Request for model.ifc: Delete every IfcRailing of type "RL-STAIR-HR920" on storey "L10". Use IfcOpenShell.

First a look at what the model holds.

```python
import ifcopenshell
import ifcopenshell.util.element

model = ifcopenshell.open("model.ifc")
print(model.schema)
storey = next(s for s in model.by_type("IfcBuildingStorey") if s.Name == "L10")
railings = [e for e in ifcopenshell.util.element.get_decomposition(storey) if e.is_a("IfcRailing")]
seen = {}
for e in railings:
    element_type = ifcopenshell.util.element.get_type(e)
    name = element_type.Name if element_type not in (None, e) else None
    seen[name] = seen.get(name, 0) + 1
for name, count in sorted(seen.items(), key=str):
    print(count, "x", name)
```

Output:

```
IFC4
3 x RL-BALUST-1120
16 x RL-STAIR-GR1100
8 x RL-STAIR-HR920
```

```python
import ifcopenshell
import ifcopenshell.api.root
import ifcopenshell.util.element

model = ifcopenshell.open("model.ifc")

storey = next(s for s in model.by_type("IfcBuildingStorey") if s.Name == "L10")
railings = [e for e in ifcopenshell.util.element.get_decomposition(storey) if e.is_a("IfcRailing")]
targets = [e for e in railings if (t := ifcopenshell.util.element.get_type(e)) not in (None, e) and t.Name == "RL-STAIR-HR920"]

for e in targets:
    ifcopenshell.api.root.remove_product(model, product=e)
print(len(targets), "removed")

model.write("model_edited.ifc")
```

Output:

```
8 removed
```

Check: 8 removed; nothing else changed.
